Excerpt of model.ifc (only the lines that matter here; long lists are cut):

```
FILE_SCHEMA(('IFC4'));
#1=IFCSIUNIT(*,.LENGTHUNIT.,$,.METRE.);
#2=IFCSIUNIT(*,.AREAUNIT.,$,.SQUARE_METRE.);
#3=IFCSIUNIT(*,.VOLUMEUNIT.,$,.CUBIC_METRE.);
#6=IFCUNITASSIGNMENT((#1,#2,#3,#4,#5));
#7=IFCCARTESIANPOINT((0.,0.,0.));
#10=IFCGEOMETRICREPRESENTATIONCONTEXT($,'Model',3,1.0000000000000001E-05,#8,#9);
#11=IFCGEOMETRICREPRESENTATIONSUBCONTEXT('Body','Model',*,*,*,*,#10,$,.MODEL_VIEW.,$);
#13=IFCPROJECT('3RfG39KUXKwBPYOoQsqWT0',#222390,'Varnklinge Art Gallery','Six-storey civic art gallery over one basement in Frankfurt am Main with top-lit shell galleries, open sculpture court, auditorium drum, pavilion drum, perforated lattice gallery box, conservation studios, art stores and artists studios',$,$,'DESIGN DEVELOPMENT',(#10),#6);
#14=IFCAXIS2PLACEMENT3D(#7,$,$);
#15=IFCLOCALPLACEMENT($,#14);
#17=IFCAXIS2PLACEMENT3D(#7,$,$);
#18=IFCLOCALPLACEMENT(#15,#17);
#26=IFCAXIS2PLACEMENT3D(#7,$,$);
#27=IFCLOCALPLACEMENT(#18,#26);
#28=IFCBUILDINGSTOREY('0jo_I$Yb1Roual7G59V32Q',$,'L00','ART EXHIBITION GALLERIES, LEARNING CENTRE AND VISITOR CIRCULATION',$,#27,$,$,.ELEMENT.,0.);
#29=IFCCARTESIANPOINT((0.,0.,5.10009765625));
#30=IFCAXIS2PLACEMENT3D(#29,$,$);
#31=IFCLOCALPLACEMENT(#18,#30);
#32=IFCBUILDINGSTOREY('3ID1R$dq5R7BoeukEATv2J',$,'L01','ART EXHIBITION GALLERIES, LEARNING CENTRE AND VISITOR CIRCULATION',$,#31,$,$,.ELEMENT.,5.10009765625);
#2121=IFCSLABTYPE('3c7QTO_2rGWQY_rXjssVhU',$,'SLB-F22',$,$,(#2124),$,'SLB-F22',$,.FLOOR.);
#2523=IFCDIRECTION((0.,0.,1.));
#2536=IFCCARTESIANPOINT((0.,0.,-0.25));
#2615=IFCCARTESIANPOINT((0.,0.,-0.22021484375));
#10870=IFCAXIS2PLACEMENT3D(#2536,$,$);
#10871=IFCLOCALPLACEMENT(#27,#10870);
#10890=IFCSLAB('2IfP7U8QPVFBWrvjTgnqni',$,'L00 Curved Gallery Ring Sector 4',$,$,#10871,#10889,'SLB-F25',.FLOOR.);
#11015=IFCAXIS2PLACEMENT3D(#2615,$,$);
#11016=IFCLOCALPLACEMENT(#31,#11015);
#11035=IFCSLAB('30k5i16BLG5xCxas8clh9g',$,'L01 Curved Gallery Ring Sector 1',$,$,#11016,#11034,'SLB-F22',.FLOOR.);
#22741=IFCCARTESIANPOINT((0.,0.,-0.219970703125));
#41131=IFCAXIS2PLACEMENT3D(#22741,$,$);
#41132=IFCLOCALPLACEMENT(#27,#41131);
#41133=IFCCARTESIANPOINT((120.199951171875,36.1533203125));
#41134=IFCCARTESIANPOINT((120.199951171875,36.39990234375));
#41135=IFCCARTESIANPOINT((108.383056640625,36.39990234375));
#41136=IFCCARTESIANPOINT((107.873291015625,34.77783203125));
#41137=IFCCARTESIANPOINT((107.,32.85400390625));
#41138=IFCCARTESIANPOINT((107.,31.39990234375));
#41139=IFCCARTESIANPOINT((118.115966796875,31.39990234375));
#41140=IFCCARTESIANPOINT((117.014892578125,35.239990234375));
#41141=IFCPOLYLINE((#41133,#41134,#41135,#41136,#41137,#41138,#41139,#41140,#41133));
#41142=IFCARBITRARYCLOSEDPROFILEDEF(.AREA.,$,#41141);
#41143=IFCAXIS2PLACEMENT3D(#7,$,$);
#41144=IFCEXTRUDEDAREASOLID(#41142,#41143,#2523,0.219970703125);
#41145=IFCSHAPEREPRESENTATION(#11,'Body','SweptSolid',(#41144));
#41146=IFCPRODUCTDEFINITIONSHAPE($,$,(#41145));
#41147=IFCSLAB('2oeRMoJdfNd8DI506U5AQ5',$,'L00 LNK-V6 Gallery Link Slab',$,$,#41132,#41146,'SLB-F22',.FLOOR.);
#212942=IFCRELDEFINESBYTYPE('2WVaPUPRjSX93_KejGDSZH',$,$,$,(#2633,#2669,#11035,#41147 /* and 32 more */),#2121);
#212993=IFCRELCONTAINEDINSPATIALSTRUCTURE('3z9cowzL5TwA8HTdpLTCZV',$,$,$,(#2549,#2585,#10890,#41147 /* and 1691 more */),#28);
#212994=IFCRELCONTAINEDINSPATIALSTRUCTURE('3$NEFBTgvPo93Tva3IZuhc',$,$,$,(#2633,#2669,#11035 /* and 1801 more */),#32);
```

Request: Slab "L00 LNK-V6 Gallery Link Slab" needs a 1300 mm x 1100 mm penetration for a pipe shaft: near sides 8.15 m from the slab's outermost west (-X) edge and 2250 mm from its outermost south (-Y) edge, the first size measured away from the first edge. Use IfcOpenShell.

```python
import numpy as np
import ifcopenshell
import ifcopenshell.api.feature
import ifcopenshell.api.geometry
import ifcopenshell.api.root
import ifcopenshell.geom
import ifcopenshell.util.placement
import ifcopenshell.util.representation
import ifcopenshell.util.shape
import ifcopenshell.util.unit

model = ifcopenshell.open("model.ifc")
unit_scale = ifcopenshell.util.unit.calculate_unit_scale(model)
settings = ifcopenshell.geom.settings()


def volume(element):
    """Net volume in cubic metres, openings subtracted."""
    shape = ifcopenshell.geom.create_shape(settings, element)
    return ifcopenshell.util.shape.get_volume(shape.geometry)


slab = model.by_guid("2oeRMoJdfNd8DI506U5AQ5")
before = volume(slab)

# Extent in the slab's own axes, in metres. The edges named are its -X and -Y sides.
slab_shape = ifcopenshell.geom.create_shape(settings, slab)
vertices = ifcopenshell.util.shape.get_vertices(slab_shape.geometry)
x_min, y_min, bottom = vertices.min(axis=0)
top = vertices[:, 2].max()

opening = ifcopenshell.api.root.create_entity(model, ifc_class="IfcOpeningElement", name="Pipe shaft opening", predefined_type="OPENING")
context = ifcopenshell.util.representation.get_context(model, "Model", "Body", "MODEL_VIEW")
width, depth = 1.3, 1.1
outline = [(0.0, 0.0), (width, 0.0), (width, depth), (0.0, depth), (0.0, 0.0)]
# Overshoot both faces by 50 mm so the cut is clean.
shape = ifcopenshell.api.geometry.add_slab_representation(
    model, context=context, depth=top - bottom + 0.1, polyline=outline
)
ifcopenshell.api.geometry.assign_representation(model, product=opening, representation=shape)

matrix = ifcopenshell.util.placement.get_local_placement(slab.ObjectPlacement)
matrix[:, 3] = matrix @ np.append(np.array([x_min + 8.15, y_min + 2.25, bottom - 0.05]) / unit_scale, 1.0)
ifcopenshell.api.geometry.edit_object_placement(model, product=opening, matrix=matrix, is_si=False)
ifcopenshell.api.feature.add_feature(model, feature=opening, element=slab)

after = volume(slab)

print(f"slab volume {before:.3f} -> {after:.3f} m3")

model.write("model_v2.ifc")
```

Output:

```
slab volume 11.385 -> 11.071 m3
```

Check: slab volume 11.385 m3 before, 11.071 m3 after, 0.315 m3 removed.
